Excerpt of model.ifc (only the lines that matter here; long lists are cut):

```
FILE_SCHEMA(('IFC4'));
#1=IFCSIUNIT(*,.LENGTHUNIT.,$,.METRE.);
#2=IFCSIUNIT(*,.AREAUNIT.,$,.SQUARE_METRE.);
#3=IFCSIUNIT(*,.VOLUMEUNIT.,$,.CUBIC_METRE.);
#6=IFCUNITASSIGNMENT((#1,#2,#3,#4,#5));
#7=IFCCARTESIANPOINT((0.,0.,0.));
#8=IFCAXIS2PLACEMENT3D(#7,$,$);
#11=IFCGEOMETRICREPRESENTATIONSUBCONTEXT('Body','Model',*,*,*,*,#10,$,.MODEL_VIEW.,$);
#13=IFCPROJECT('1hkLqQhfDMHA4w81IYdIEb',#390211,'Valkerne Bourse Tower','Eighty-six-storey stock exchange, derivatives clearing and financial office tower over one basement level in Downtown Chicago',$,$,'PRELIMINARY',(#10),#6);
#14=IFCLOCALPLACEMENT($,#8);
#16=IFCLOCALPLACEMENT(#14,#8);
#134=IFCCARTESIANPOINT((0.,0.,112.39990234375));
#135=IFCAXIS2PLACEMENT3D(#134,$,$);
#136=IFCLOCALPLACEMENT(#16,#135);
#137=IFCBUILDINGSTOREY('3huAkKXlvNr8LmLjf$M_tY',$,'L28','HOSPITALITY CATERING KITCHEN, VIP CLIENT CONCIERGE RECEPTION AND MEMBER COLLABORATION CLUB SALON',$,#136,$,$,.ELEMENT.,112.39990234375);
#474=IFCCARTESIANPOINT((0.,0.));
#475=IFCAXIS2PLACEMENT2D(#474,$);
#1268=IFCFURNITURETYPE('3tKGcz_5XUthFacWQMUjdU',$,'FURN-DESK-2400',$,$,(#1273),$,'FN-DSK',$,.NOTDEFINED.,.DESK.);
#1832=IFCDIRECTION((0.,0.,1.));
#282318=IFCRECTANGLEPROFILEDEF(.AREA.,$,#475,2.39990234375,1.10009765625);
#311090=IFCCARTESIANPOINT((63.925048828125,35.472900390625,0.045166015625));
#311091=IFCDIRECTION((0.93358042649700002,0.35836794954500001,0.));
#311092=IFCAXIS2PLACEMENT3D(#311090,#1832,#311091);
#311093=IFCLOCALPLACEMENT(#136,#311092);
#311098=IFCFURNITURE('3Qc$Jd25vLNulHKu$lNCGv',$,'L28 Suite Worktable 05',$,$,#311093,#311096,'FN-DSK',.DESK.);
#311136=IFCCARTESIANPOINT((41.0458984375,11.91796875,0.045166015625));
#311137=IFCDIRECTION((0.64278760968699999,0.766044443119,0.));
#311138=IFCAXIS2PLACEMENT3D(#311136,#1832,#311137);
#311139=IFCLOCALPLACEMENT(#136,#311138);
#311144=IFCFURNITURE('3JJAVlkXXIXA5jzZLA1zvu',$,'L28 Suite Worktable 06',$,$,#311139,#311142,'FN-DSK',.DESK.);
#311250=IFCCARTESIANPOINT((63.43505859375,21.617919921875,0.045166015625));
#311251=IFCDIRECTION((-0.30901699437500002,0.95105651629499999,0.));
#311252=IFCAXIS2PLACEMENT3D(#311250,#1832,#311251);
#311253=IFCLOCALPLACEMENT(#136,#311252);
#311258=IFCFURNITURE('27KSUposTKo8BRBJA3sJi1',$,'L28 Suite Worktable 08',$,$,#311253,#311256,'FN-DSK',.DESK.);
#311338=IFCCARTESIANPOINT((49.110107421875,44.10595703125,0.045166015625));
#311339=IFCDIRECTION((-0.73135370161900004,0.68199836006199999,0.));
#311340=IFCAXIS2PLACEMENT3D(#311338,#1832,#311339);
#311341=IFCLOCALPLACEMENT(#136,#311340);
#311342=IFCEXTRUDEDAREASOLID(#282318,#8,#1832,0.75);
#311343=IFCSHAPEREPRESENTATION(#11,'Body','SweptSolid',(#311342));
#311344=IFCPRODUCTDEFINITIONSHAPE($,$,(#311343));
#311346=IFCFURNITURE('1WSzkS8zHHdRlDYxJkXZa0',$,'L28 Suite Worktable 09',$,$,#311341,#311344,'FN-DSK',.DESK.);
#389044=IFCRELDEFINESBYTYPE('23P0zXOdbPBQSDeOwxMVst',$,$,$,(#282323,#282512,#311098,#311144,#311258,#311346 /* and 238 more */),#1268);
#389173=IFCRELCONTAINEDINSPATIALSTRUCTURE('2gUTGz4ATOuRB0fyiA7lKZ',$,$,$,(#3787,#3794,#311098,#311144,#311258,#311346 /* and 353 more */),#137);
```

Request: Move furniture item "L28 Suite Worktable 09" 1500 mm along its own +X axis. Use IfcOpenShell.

```python
import ifcopenshell
import ifcopenshell.api.geometry
import ifcopenshell.util.placement
import ifcopenshell.util.unit

model = ifcopenshell.open("model.ifc")
unit_scale = ifcopenshell.util.unit.calculate_unit_scale(model)

item = model.by_guid("1WSzkS8zHHdRlDYxJkXZa0")
matrix = ifcopenshell.util.placement.get_local_placement(item.ObjectPlacement)
matrix[:3, 3] += matrix[:3, 0] * 1.5 / unit_scale
ifcopenshell.api.geometry.edit_object_placement(model, product=item, matrix=matrix, is_si=False)

print(ifcopenshell.util.placement.get_local_placement(item.ObjectPlacement).round(3) + 0.0)

model.write("model_v2.ifc")
```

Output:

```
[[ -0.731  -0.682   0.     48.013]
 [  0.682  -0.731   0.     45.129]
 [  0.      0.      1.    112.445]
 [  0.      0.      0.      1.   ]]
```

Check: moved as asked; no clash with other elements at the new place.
